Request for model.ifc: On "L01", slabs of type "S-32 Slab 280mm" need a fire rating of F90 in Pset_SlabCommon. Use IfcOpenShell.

First a look at what the model holds.

```python
import ifcopenshell
import ifcopenshell.util.element

model = ifcopenshell.open("model.ifc")
print(model.schema)
storey = next(s for s in model.by_type("IfcBuildingStorey") if s.Name == "L01")
slabs = [e for e in ifcopenshell.util.element.get_decomposition(storey) if e.is_a("IfcSlab")]
seen = {}
for e in slabs:
    element_type = ifcopenshell.util.element.get_type(e)
    key = (element_type.Name if element_type != e and element_type else None, ifcopenshell.util.element.get_pset(e, "Pset_SlabCommon", "FireRating"))
    seen[key] = seen.get(key, 0) + 1
for (name, value), count in sorted(seen.items(), key=str):
    print(count, "x", name, "|", value)
```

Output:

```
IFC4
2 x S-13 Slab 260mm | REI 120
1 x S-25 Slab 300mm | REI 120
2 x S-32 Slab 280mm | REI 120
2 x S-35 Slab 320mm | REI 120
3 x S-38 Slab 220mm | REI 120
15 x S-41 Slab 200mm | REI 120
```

```python
import ifcopenshell
import ifcopenshell.api.pset
import ifcopenshell.util.element

model = ifcopenshell.open("model.ifc")

storey = next(s for s in model.by_type("IfcBuildingStorey") if s.Name == "L01")
slabs = [e for e in ifcopenshell.util.element.get_decomposition(storey) if e.is_a("IfcSlab")]

count = 0
for e in slabs:
    element_type = ifcopenshell.util.element.get_type(e)
    if element_type in (None, e) or element_type.Name != "S-32 Slab 280mm":
        continue
    # add_pset returns the element's existing set when there is one.
    pset = ifcopenshell.api.pset.add_pset(model, product=e, name="Pset_SlabCommon")
    ifcopenshell.api.pset.edit_pset(model, pset=pset, properties={"FireRating": "F90"})
    count += 1

print(count, "slabs updated")

model.write("model_updated.ifc")
```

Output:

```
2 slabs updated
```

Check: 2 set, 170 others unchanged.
